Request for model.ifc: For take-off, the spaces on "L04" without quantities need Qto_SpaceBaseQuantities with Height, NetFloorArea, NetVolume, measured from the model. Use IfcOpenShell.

First a look at what the model holds.

```python
import ifcopenshell
import ifcopenshell.util.element
import ifcopenshell.util.unit

model = ifcopenshell.open("model.ifc")
print(model.schema)
for unit_type in ("LENGTHUNIT", "AREAUNIT", "VOLUMEUNIT"):
    print(unit_type, ifcopenshell.util.unit.calculate_unit_scale(model, unit_type))
storey = next(s for s in model.by_type("IfcBuildingStorey") if s.Name == "L04")
spaces = [e for e in ifcopenshell.util.element.get_decomposition(storey) if e.is_a("IfcSpace")]
for e in sorted(spaces, key=lambda e: e.id()):
    print(e.id(), e.is_a(), e.Name, list(ifcopenshell.util.element.get_psets(e, qtos_only=True)), sep=" | ")
```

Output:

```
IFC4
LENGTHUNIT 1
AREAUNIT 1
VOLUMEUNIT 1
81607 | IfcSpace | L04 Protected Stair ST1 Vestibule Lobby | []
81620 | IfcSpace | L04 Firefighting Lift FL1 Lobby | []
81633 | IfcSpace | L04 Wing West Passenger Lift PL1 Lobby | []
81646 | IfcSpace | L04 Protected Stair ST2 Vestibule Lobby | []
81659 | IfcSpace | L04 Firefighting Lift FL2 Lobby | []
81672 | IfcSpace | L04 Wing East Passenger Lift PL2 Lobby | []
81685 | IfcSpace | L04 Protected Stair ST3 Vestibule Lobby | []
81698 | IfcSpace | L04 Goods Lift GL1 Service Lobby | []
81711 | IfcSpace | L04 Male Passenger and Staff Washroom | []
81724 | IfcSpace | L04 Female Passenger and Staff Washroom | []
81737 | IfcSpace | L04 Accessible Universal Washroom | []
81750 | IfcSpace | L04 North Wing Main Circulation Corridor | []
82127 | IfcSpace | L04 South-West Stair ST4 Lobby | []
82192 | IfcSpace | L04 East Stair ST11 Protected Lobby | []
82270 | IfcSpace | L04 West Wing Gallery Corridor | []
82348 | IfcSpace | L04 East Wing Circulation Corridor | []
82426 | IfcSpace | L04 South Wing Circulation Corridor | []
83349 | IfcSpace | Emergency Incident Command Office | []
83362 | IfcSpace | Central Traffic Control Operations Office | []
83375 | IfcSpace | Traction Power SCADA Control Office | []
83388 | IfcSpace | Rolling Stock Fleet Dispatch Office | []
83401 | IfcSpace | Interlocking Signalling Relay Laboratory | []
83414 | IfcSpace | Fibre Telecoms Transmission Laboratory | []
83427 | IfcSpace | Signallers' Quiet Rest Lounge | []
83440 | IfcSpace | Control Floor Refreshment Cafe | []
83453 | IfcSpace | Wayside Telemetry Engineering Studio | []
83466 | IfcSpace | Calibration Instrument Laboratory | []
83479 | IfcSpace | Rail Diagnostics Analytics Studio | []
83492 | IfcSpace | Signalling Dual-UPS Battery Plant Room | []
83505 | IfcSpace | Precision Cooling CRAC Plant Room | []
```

```python
import ifcopenshell
import ifcopenshell.api.pset
import ifcopenshell.geom
import ifcopenshell.util.element
import ifcopenshell.util.shape
import ifcopenshell.util.unit

model = ifcopenshell.open("model.ifc")
unit_scale = ifcopenshell.util.unit.calculate_unit_scale(model)
area_scale = ifcopenshell.util.unit.calculate_unit_scale(model, "AREAUNIT")
volume_scale = ifcopenshell.util.unit.calculate_unit_scale(model, "VOLUMEUNIT")
settings = ifcopenshell.geom.settings()

storey = next(s for s in model.by_type("IfcBuildingStorey") if s.Name == "L04")
spaces = [e for e in ifcopenshell.util.element.get_decomposition(storey) if e.is_a("IfcSpace")]

for e in sorted(spaces, key=lambda e: e.id()):
    if ifcopenshell.util.element.get_psets(e, qtos_only=True, should_inherit=False):
        continue
    # Geometry comes back in metres, in the element's own axes.
    shape = ifcopenshell.geom.create_shape(settings, e)
    values = {
        "Height": ifcopenshell.util.shape.get_z(shape.geometry) / unit_scale,
        "NetFloorArea": ifcopenshell.util.shape.get_footprint_area(shape.geometry) / area_scale,
        "NetVolume": ifcopenshell.util.shape.get_volume(shape.geometry) / volume_scale,
    }
    qto = ifcopenshell.api.pset.add_qto(model, product=e, name="Qto_SpaceBaseQuantities")
    ifcopenshell.api.pset.edit_qto(model, qto=qto, properties=values)
    print(e.id(), {k: round(v, 3) for k, v in values.items()})

model.write("model_edited.ifc")
```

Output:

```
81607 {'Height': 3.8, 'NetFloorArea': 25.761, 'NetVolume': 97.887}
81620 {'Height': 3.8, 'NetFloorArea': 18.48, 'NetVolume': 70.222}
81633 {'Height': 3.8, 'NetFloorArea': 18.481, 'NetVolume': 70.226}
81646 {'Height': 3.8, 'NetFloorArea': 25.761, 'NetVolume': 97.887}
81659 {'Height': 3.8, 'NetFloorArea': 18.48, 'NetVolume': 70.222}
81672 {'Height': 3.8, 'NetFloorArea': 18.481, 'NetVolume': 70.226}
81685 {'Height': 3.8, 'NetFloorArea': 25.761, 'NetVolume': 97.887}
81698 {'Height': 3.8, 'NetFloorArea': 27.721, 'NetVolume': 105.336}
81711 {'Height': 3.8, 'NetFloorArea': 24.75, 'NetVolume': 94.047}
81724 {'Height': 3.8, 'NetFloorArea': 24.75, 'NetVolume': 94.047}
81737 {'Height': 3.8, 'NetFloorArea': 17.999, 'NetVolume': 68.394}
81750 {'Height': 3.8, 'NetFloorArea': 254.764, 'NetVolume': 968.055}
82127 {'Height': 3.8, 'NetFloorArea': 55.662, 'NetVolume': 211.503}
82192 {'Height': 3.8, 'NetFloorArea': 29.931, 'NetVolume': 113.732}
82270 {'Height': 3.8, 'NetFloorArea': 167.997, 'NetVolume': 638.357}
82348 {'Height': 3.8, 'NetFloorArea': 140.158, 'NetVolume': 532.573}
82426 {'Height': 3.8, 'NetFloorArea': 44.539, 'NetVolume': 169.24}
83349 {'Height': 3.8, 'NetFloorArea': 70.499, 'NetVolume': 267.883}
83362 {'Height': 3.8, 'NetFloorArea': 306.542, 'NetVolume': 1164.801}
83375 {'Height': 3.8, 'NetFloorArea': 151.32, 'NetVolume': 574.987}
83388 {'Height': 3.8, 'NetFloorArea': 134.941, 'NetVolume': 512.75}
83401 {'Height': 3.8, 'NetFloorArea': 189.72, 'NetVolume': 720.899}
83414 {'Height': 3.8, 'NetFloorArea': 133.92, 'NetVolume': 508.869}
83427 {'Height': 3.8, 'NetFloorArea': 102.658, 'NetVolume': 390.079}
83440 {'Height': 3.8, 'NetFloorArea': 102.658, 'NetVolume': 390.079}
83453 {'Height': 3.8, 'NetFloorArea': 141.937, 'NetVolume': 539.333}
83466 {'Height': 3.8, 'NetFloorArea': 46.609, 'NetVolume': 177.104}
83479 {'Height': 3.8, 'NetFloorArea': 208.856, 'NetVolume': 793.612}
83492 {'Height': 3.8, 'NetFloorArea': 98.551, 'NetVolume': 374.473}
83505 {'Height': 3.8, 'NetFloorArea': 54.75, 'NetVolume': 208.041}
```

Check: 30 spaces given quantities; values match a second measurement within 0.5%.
